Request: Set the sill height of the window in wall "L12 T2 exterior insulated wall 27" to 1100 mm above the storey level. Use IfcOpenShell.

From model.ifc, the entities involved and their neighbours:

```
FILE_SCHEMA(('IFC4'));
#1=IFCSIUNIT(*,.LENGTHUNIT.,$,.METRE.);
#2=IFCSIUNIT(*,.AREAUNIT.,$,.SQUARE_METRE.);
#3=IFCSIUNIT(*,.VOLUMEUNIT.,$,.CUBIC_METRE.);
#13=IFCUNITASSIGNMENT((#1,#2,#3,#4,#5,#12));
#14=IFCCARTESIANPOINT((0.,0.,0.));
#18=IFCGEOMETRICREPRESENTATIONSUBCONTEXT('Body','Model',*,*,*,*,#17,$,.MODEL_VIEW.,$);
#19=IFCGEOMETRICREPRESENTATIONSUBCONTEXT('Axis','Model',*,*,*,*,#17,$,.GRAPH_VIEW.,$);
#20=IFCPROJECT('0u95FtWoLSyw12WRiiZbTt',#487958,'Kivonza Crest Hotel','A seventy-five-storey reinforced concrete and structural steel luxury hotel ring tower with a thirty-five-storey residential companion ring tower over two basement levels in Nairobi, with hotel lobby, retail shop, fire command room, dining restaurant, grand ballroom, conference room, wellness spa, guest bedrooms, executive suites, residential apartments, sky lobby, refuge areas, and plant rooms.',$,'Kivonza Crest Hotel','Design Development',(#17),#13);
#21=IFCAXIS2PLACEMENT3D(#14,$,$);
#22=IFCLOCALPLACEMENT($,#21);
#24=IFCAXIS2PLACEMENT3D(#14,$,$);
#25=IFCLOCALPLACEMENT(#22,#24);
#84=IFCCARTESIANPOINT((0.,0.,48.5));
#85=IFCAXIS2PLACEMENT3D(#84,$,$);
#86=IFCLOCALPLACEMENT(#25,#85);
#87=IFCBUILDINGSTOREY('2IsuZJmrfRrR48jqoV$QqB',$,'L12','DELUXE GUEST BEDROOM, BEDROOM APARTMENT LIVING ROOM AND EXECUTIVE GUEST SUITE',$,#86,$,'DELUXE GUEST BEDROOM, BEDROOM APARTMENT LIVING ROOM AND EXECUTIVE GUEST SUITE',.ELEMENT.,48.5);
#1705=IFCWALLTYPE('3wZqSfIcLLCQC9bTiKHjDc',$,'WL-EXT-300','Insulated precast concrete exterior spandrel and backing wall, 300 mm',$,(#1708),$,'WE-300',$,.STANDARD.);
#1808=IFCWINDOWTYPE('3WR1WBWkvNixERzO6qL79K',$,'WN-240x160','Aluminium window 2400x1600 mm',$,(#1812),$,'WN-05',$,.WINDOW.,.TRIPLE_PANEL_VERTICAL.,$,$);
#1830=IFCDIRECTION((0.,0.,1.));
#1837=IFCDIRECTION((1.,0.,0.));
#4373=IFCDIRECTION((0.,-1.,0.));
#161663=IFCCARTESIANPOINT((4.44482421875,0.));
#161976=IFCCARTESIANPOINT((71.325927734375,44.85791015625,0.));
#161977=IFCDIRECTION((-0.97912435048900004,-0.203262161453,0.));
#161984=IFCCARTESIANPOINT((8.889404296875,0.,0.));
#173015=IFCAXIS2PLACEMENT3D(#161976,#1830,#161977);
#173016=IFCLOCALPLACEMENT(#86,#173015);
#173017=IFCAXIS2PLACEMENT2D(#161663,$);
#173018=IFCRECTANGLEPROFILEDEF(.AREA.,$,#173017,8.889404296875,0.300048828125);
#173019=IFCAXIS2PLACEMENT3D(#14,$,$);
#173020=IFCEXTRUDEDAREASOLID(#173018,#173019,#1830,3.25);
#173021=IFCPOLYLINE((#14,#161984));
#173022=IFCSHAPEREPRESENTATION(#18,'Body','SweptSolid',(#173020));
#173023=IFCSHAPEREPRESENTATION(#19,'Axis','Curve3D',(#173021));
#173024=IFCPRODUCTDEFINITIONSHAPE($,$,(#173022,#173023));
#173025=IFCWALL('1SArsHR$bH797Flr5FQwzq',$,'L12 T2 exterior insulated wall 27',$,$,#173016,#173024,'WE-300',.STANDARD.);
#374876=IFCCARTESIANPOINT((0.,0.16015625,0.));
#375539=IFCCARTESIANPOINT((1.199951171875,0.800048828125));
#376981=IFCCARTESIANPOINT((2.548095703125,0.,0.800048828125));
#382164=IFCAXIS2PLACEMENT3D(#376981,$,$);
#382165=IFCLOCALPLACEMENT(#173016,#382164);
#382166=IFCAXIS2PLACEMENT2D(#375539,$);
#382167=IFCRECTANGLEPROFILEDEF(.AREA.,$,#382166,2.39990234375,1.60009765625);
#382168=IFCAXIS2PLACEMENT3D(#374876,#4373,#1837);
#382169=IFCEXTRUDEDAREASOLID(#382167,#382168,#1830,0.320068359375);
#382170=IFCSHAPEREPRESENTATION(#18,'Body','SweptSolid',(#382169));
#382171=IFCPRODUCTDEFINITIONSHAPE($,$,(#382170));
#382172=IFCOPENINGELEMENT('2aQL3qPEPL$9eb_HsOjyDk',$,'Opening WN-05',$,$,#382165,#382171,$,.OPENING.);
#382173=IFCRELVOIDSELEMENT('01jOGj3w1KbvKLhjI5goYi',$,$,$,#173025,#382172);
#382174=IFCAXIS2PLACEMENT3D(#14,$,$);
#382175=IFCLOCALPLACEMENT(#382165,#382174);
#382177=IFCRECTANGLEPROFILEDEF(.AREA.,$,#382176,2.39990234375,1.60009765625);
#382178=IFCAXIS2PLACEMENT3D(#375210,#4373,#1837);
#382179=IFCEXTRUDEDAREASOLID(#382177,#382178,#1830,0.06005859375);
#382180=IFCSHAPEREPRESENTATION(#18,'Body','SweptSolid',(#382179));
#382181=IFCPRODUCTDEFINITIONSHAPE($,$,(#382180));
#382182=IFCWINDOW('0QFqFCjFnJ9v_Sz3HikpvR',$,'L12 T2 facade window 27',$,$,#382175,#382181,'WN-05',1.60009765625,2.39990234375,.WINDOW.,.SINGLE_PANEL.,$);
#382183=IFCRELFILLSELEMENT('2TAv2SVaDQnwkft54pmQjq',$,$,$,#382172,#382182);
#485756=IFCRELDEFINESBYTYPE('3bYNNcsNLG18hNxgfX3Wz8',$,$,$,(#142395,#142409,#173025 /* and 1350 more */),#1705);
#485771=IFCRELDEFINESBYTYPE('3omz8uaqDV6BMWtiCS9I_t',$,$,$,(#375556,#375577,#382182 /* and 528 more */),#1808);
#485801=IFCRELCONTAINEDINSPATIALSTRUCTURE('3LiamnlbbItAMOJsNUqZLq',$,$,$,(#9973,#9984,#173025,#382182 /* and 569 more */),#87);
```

```python
import numpy as np
import ifcopenshell
import ifcopenshell.api.geometry
import ifcopenshell.geom
import ifcopenshell.util.element
import ifcopenshell.util.placement
import ifcopenshell.util.shape
import ifcopenshell.util.unit

model = ifcopenshell.open("model.ifc")
unit_scale = ifcopenshell.util.unit.calculate_unit_scale(model)

window = model.by_id(382182)
opening = window.FillsVoids[0].RelatingOpeningElement
storey = ifcopenshell.util.element.get_container(window, ifc_class="IfcBuildingStorey")
level = ifcopenshell.util.placement.get_local_placement(storey.ObjectPlacement)[2, 3]

# The opening's origin need not be at the sill, so measure its lowest point.
shape = ifcopenshell.geom.create_shape(ifcopenshell.geom.settings(), opening)
bottom = ifcopenshell.util.shape.get_shape_bottom_elevation(shape, shape.geometry) / unit_scale
dz = level + 1.1 / unit_scale - bottom

shift = np.array([0.0, 0.0, dz])
# The window is placed relative to its opening, so it follows when the opening moves.
matrix = ifcopenshell.util.placement.get_local_placement(opening.ObjectPlacement)
matrix[:3, 3] += shift
ifcopenshell.api.geometry.edit_object_placement(
    model, product=opening, matrix=matrix, is_si=False, should_transform_children=True
)

print(f"moved by {dz * unit_scale:+.3f} m")

model.write("model_updated.ifc")
```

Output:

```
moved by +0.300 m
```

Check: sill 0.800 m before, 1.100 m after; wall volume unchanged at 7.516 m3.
